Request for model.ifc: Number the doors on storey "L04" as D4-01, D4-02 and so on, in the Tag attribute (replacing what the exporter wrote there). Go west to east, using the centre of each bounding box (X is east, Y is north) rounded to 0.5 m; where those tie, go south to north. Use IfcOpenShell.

First a look at what the model holds.

```python
import ifcopenshell
import ifcopenshell.util.element
import ifcopenshell.util.placement

model = ifcopenshell.open("model.ifc")
print(model.schema)
storey = next(s for s in model.by_type("IfcBuildingStorey") if s.Name == "L04")
doors = [e for e in ifcopenshell.util.element.get_decomposition(storey) if e.is_a("IfcDoor")]
for e in sorted(doors, key=lambda e: e.id()):
    origin = ifcopenshell.util.placement.get_local_placement(e.ObjectPlacement)[:3, 3]
    print(e.id(), e.Tag, e.Name, origin.round(2) + 0.0, sep=" | ")
```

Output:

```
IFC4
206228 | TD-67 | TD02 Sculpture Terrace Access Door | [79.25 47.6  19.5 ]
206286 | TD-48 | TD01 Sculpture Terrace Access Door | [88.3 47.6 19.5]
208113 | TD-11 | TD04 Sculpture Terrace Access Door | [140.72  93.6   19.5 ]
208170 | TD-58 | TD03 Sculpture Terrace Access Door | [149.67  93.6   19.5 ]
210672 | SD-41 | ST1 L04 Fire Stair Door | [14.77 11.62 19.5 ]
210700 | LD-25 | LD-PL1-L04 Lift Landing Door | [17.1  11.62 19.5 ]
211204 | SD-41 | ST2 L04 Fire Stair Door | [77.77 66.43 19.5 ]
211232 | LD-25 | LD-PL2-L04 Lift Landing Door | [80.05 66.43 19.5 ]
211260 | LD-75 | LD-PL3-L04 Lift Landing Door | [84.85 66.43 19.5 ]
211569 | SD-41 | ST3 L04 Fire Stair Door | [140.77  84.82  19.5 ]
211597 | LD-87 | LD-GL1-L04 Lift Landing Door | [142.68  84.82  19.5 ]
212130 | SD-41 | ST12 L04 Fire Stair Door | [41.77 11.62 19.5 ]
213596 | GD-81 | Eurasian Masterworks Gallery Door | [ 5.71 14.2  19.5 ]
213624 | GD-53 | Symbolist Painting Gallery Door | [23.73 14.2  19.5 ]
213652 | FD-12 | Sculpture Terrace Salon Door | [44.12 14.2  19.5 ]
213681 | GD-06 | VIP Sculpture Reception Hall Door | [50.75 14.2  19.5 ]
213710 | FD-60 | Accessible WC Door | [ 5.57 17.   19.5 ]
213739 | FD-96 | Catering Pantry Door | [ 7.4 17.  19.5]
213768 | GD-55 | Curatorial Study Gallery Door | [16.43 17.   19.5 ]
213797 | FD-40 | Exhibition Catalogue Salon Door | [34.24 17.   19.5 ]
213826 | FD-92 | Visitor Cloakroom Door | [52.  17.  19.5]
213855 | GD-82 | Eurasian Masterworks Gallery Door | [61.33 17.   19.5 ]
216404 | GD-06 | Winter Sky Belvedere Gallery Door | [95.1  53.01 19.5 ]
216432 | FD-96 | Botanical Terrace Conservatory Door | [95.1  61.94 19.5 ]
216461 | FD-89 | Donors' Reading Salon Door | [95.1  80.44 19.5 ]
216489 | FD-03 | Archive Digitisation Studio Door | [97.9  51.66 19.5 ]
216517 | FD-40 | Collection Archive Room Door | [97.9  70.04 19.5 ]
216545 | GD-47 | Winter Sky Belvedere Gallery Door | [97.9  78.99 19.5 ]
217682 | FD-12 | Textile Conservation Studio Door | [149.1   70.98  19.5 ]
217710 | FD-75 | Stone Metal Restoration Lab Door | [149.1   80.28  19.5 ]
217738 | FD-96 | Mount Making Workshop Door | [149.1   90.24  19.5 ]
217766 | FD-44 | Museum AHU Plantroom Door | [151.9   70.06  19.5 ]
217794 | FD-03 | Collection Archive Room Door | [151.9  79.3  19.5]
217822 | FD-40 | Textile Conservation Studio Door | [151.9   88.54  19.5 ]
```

```python
import ifcopenshell
import ifcopenshell.geom
import ifcopenshell.util.element
import ifcopenshell.util.shape

model = ifcopenshell.open("model.ifc")
settings = ifcopenshell.geom.settings()
settings.set("use-world-coords", True)


def centre(element):
    shape = ifcopenshell.geom.create_shape(settings, element)
    return ifcopenshell.util.shape.get_bbox_centroid(shape.geometry)


storey = next(s for s in model.by_type("IfcBuildingStorey") if s.Name == "L04")
doors = [e for e in ifcopenshell.util.element.get_decomposition(storey) if e.is_a("IfcDoor")]

# Insertion points can sit at a corner or the storey origin, so sort by the geometry (in metres).
centres = {e: centre(e) for e in doors}
doors.sort(key=lambda e: (round(centres[e][0] / 0.5), centres[e][1]))

for i, e in enumerate(doors, start=1):
    number = f"D4-{i:02d}"
    e.Tag = number
    print(e.id(), number)

model.write("model_v2.ifc")
```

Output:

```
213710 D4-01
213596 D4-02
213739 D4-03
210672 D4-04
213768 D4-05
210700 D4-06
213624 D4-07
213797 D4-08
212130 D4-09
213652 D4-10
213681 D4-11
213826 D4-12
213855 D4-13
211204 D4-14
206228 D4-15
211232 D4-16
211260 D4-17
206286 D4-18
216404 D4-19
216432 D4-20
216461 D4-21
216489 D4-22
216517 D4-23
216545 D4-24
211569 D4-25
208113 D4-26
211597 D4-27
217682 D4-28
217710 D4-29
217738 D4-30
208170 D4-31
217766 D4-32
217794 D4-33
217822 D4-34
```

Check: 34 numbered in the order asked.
